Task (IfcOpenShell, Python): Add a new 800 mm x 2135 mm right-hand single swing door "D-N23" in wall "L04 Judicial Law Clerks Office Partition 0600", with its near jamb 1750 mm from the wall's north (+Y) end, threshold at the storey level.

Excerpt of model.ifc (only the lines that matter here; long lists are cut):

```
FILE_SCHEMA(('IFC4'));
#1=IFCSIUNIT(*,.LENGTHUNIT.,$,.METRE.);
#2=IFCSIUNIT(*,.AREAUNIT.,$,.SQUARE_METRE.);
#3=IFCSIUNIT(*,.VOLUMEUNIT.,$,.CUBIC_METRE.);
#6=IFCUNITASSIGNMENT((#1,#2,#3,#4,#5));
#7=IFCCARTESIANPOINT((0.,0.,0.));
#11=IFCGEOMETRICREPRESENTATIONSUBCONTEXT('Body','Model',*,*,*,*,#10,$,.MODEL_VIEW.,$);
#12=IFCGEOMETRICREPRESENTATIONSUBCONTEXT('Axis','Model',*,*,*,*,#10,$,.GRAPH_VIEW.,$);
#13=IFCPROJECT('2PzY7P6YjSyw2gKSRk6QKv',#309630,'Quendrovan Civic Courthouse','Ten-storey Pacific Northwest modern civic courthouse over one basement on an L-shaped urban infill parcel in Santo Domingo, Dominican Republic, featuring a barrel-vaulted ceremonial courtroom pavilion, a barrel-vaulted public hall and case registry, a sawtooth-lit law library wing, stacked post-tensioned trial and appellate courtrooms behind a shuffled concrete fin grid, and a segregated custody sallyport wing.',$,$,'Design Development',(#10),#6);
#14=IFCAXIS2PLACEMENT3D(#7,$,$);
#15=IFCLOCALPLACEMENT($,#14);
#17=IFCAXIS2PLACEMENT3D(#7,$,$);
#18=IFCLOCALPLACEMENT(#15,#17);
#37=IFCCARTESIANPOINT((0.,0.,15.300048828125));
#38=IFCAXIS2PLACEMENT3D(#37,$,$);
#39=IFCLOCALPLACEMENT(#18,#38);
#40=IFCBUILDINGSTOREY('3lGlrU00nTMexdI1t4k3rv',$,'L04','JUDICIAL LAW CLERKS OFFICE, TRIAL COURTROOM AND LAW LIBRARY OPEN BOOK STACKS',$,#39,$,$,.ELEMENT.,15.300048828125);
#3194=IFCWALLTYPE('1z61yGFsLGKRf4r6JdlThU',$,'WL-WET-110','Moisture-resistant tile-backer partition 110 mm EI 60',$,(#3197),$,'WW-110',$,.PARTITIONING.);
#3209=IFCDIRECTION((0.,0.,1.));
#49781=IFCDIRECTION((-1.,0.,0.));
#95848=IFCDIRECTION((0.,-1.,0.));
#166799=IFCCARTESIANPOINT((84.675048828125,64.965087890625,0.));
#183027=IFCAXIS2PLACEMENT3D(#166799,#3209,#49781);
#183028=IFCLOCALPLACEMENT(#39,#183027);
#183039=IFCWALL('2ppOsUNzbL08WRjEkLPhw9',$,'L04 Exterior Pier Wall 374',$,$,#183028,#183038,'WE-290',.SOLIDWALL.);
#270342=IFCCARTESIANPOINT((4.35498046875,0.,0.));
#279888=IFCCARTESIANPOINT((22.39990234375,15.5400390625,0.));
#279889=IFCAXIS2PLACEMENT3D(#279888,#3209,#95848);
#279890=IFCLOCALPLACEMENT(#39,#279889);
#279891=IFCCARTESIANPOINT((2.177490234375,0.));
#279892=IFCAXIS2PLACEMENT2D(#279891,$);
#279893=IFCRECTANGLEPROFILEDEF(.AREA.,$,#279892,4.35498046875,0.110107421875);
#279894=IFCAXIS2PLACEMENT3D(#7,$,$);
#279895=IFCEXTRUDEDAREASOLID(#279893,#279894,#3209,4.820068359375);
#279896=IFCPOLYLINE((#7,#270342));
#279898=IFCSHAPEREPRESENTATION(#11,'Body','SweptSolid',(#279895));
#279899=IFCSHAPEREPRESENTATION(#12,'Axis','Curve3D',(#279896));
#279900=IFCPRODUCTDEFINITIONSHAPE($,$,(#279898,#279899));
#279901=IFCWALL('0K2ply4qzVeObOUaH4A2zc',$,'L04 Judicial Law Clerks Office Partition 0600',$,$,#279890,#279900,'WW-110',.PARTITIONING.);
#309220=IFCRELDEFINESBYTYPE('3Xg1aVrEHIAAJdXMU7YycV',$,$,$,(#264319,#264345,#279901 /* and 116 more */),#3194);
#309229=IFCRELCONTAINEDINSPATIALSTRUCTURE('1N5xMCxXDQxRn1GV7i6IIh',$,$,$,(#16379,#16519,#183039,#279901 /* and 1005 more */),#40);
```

```python
import numpy as np
import ifcopenshell
import ifcopenshell.api.feature
import ifcopenshell.api.geometry
import ifcopenshell.api.root
import ifcopenshell.api.spatial
import ifcopenshell.geom
import ifcopenshell.util.element
import ifcopenshell.util.placement
import ifcopenshell.util.representation
import ifcopenshell.util.shape
import ifcopenshell.util.unit

model = ifcopenshell.open("model.ifc")
unit_scale = ifcopenshell.util.unit.calculate_unit_scale(model)
settings = ifcopenshell.geom.settings()


def volume(element):
    """Net volume in cubic metres, openings subtracted."""
    shape = ifcopenshell.geom.create_shape(settings, element)
    return ifcopenshell.util.shape.get_volume(shape.geometry)


wall = model.by_guid("0K2ply4qzVeObOUaH4A2zc")
storey = ifcopenshell.util.element.get_container(wall, ifc_class="IfcBuildingStorey")
context = ifcopenshell.util.representation.get_context(model, "Model", "Body", "MODEL_VIEW")
before = volume(wall)

width, height, from_end, sill = 0.8, 2.135, 1.75, 0.0  # metres

# The wall runs along its own X axis, and the end named is its -X end.
wall_shape = ifcopenshell.geom.create_shape(settings, wall)
x, y, z = ifcopenshell.util.shape.get_vertices(wall_shape.geometry).T
start = x.min() + from_end
face, thickness = float(y.min()), float(y.max() - y.min())
wall_matrix = ifcopenshell.util.placement.get_local_placement(wall.ObjectPlacement)
level = ifcopenshell.util.placement.get_local_placement(storey.ObjectPlacement)[2, 3]


def in_wall(x, y):
    """Placement at x, y metres in the wall's axes, at sill height."""
    matrix = wall_matrix.copy()
    matrix[:, 3] = wall_matrix @ np.array([x / unit_scale, y / unit_scale, 0.0, 1.0])
    matrix[2, 3] = level + sill / unit_scale
    return matrix


# Opening: a box that overshoots both wall faces by 50 mm.
opening = ifcopenshell.api.root.create_entity(model, ifc_class="IfcOpeningElement", predefined_type="OPENING")
box = ifcopenshell.api.geometry.add_wall_representation(
    model, context=context, length=width, height=height, thickness=thickness + 0.1
)
ifcopenshell.api.geometry.assign_representation(model, product=opening, representation=box)
ifcopenshell.api.geometry.edit_object_placement(model, product=opening, matrix=in_wall(start, face - 0.05), is_si=False)
ifcopenshell.api.feature.add_feature(model, feature=opening, element=wall)

door = ifcopenshell.api.root.create_entity(model, ifc_class="IfcDoor", name="D-N23", predefined_type="DOOR")
door.OverallWidth, door.OverallHeight = width / unit_scale, height / unit_scale
door.OperationType = "SINGLE_SWING_RIGHT"
body = ifcopenshell.api.geometry.add_door_representation(
    model,
    context=context,
    overall_width=door.OverallWidth,
    overall_height=door.OverallHeight,
    operation_type="SINGLE_SWING_RIGHT",
    lining_properties={"LiningDepth": thickness / unit_scale, "ThresholdDepth": thickness / unit_scale},
)
ifcopenshell.api.geometry.assign_representation(model, product=door, representation=body)
ifcopenshell.api.spatial.assign_container(model, products=[door], relating_structure=storey)
ifcopenshell.api.feature.add_filling(model, opening=opening, element=door)

# The lining spans the wall, so the door starts at the wall face.
ifcopenshell.api.geometry.edit_object_placement(model, product=door, matrix=in_wall(start, face), is_si=False)

after = volume(wall)

print(f"wall volume {before:.3f} -> {after:.3f} m3")

model.write("model_v2.ifc")
```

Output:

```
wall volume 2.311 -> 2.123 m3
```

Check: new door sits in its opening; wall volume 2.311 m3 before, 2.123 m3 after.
